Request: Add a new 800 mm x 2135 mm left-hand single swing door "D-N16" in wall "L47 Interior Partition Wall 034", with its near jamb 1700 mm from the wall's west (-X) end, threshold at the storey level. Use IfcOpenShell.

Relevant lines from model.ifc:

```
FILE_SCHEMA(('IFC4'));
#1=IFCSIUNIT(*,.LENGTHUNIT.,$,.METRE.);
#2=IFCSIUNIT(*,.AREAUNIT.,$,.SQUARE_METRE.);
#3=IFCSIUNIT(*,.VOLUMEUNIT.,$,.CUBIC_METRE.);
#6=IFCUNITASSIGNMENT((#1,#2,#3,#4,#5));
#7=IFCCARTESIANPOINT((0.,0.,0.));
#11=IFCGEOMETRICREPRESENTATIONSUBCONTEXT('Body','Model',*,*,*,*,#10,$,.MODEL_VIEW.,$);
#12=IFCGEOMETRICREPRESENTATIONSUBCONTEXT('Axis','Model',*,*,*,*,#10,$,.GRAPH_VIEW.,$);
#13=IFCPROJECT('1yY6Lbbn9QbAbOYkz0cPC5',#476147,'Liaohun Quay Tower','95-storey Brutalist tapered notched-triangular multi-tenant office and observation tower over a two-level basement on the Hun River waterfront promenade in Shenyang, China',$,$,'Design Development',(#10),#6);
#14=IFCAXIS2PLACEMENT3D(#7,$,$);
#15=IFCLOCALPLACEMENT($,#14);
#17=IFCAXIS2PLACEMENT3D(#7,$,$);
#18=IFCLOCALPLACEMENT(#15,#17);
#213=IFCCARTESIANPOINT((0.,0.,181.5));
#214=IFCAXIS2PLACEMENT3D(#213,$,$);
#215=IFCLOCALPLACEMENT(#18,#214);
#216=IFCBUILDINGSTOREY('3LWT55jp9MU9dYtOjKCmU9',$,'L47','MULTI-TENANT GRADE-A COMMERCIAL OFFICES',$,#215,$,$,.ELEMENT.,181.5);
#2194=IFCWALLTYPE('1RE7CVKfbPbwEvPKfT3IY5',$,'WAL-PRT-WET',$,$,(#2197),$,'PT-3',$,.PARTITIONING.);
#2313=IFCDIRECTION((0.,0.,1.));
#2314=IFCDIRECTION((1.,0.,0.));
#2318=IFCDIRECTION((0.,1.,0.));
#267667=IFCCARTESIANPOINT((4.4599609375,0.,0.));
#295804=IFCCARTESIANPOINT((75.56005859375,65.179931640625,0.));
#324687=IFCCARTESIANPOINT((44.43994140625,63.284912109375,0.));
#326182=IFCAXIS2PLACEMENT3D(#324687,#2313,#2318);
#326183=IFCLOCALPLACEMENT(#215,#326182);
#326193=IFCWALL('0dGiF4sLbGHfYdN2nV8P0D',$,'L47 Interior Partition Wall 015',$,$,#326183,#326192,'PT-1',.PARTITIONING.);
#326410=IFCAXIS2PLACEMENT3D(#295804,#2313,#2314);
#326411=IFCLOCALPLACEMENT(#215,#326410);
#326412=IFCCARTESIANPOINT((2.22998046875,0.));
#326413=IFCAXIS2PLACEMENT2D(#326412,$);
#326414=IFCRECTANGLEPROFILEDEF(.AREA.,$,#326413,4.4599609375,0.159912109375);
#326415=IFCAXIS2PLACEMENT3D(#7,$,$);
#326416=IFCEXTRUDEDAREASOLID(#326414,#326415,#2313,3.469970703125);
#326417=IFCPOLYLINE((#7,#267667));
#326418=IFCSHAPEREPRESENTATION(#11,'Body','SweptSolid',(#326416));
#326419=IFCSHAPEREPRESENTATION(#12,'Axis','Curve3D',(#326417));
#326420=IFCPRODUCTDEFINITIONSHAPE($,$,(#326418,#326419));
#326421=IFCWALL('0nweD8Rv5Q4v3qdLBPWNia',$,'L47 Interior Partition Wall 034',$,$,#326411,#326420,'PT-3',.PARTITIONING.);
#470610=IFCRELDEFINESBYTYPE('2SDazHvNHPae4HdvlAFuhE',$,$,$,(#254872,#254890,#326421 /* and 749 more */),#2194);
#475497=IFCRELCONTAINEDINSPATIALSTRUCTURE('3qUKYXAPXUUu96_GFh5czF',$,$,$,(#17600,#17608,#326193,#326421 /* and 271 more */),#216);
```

```python
import numpy as np
import ifcopenshell
import ifcopenshell.api.feature
import ifcopenshell.api.geometry
import ifcopenshell.api.root
import ifcopenshell.api.spatial
import ifcopenshell.geom
import ifcopenshell.util.element
import ifcopenshell.util.placement
import ifcopenshell.util.representation
import ifcopenshell.util.shape
import ifcopenshell.util.unit

model = ifcopenshell.open("model.ifc")
unit_scale = ifcopenshell.util.unit.calculate_unit_scale(model)
settings = ifcopenshell.geom.settings()


def volume(element):
    """Net volume in cubic metres, openings subtracted."""
    shape = ifcopenshell.geom.create_shape(settings, element)
    return ifcopenshell.util.shape.get_volume(shape.geometry)


wall = model.by_guid("0nweD8Rv5Q4v3qdLBPWNia")
storey = ifcopenshell.util.element.get_container(wall, ifc_class="IfcBuildingStorey")
context = ifcopenshell.util.representation.get_context(model, "Model", "Body", "MODEL_VIEW")
before = volume(wall)

width, height, from_end, sill = 0.8, 2.135, 1.7, 0.0  # metres

# The wall runs along its own X axis, and the end named is its -X end.
wall_shape = ifcopenshell.geom.create_shape(settings, wall)
x, y, z = ifcopenshell.util.shape.get_vertices(wall_shape.geometry).T
start = x.min() + from_end
face, thickness = float(y.min()), float(y.max() - y.min())
wall_matrix = ifcopenshell.util.placement.get_local_placement(wall.ObjectPlacement)
level = ifcopenshell.util.placement.get_local_placement(storey.ObjectPlacement)[2, 3]


def in_wall(x, y):
    """Placement at x, y metres in the wall's axes, at sill height."""
    matrix = wall_matrix.copy()
    matrix[:, 3] = wall_matrix @ np.array([x / unit_scale, y / unit_scale, 0.0, 1.0])
    matrix[2, 3] = level + sill / unit_scale
    return matrix


# Opening: a box that overshoots both wall faces by 50 mm.
opening = ifcopenshell.api.root.create_entity(model, ifc_class="IfcOpeningElement", predefined_type="OPENING")
box = ifcopenshell.api.geometry.add_wall_representation(
    model, context=context, length=width, height=height, thickness=thickness + 0.1
)
ifcopenshell.api.geometry.assign_representation(model, product=opening, representation=box)
ifcopenshell.api.geometry.edit_object_placement(model, product=opening, matrix=in_wall(start, face - 0.05), is_si=False)
ifcopenshell.api.feature.add_feature(model, feature=opening, element=wall)

door = ifcopenshell.api.root.create_entity(model, ifc_class="IfcDoor", name="D-N16", predefined_type="DOOR")
door.OverallWidth, door.OverallHeight = width / unit_scale, height / unit_scale
door.OperationType = "SINGLE_SWING_LEFT"
body = ifcopenshell.api.geometry.add_door_representation(
    model,
    context=context,
    overall_width=door.OverallWidth,
    overall_height=door.OverallHeight,
    operation_type="SINGLE_SWING_LEFT",
    lining_properties={"LiningDepth": thickness / unit_scale, "ThresholdDepth": thickness / unit_scale},
)
ifcopenshell.api.geometry.assign_representation(model, product=door, representation=body)
ifcopenshell.api.spatial.assign_container(model, products=[door], relating_structure=storey)
ifcopenshell.api.feature.add_filling(model, opening=opening, element=door)

# The lining spans the wall, so the door starts at the wall face.
ifcopenshell.api.geometry.edit_object_placement(model, product=door, matrix=in_wall(start, face), is_si=False)

after = volume(wall)

print(f"wall volume {before:.3f} -> {after:.3f} m3")

model.write("model_v2.ifc")
```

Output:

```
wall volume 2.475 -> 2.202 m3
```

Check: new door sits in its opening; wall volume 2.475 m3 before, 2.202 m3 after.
